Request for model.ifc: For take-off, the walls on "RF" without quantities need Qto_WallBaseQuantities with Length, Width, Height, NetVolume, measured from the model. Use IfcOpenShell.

First a look at what the model holds.

```python
import ifcopenshell
import ifcopenshell.util.element
import ifcopenshell.util.unit

model = ifcopenshell.open("model.ifc")
print(model.schema)
for unit_type in ("LENGTHUNIT", "AREAUNIT", "VOLUMEUNIT"):
    print(unit_type, ifcopenshell.util.unit.calculate_unit_scale(model, unit_type))
storey = next(s for s in model.by_type("IfcBuildingStorey") if s.Name == "RF")
walls = [e for e in ifcopenshell.util.element.get_decomposition(storey) if e.is_a("IfcWall")]
for e in sorted(walls, key=lambda e: e.id()):
    print(e.id(), e.is_a(), e.Name, list(ifcopenshell.util.element.get_psets(e, qtos_only=True)), sep=" | ")
```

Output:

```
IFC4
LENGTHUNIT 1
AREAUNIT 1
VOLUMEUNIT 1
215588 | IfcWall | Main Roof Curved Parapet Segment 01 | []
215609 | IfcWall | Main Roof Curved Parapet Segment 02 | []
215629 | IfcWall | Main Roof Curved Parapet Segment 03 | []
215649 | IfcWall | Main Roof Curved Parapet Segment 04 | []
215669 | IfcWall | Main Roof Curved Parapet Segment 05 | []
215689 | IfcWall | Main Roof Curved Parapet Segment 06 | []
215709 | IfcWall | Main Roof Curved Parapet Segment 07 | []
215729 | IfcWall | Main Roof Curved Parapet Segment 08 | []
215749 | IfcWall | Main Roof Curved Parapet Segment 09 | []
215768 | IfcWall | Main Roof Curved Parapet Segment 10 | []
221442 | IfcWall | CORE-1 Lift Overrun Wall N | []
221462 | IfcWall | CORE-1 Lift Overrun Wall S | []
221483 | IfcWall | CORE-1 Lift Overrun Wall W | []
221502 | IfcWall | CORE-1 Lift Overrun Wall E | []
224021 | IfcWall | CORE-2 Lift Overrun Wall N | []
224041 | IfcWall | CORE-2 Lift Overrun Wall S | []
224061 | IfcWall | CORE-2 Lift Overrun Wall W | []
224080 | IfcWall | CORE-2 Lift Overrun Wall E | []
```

```python
import ifcopenshell
import ifcopenshell.api.pset
import ifcopenshell.geom
import ifcopenshell.util.element
import ifcopenshell.util.shape
import ifcopenshell.util.unit

model = ifcopenshell.open("model.ifc")
unit_scale = ifcopenshell.util.unit.calculate_unit_scale(model)
volume_scale = ifcopenshell.util.unit.calculate_unit_scale(model, "VOLUMEUNIT")
settings = ifcopenshell.geom.settings()

storey = next(s for s in model.by_type("IfcBuildingStorey") if s.Name == "RF")
walls = [e for e in ifcopenshell.util.element.get_decomposition(storey) if e.is_a("IfcWall")]

for e in sorted(walls, key=lambda e: e.id()):
    if ifcopenshell.util.element.get_psets(e, qtos_only=True, should_inherit=False):
        continue
    # Geometry comes back in metres, in the element's own axes.
    shape = ifcopenshell.geom.create_shape(settings, e)
    values = {
        "Length": ifcopenshell.util.shape.get_x(shape.geometry) / unit_scale,
        "Width": ifcopenshell.util.shape.get_y(shape.geometry) / unit_scale,
        "Height": ifcopenshell.util.shape.get_z(shape.geometry) / unit_scale,
        "NetVolume": ifcopenshell.util.shape.get_volume(shape.geometry) / volume_scale,
    }
    qto = ifcopenshell.api.pset.add_qto(model, product=e, name="Qto_WallBaseQuantities")
    ifcopenshell.api.pset.edit_qto(model, qto=qto, properties=values)
    print(e.id(), {k: round(v, 3) for k, v in values.items()})

model.write("model_updated.ifc")
```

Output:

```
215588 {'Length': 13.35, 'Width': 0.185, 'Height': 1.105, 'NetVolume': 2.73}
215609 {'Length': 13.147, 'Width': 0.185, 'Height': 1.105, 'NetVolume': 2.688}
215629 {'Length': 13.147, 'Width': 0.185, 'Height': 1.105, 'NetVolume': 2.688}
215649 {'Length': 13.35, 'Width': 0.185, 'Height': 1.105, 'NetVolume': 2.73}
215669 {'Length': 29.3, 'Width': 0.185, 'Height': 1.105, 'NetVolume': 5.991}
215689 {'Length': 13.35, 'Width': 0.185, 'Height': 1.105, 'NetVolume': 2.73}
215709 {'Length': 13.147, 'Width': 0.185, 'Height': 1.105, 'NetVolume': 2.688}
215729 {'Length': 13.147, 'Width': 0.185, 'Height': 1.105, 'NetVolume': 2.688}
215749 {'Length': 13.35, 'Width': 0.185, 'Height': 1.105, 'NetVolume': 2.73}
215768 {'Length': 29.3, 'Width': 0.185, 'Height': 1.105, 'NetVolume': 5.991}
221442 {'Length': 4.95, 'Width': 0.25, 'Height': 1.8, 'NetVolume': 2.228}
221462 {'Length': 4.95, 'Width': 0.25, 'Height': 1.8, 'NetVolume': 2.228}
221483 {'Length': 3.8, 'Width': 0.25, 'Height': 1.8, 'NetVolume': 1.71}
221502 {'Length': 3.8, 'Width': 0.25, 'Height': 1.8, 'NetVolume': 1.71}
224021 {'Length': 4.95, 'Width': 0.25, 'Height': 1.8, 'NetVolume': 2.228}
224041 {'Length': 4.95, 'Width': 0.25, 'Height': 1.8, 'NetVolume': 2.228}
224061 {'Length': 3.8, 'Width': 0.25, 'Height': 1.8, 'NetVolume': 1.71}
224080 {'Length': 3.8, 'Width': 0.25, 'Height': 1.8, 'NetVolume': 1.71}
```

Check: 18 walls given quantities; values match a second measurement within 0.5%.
